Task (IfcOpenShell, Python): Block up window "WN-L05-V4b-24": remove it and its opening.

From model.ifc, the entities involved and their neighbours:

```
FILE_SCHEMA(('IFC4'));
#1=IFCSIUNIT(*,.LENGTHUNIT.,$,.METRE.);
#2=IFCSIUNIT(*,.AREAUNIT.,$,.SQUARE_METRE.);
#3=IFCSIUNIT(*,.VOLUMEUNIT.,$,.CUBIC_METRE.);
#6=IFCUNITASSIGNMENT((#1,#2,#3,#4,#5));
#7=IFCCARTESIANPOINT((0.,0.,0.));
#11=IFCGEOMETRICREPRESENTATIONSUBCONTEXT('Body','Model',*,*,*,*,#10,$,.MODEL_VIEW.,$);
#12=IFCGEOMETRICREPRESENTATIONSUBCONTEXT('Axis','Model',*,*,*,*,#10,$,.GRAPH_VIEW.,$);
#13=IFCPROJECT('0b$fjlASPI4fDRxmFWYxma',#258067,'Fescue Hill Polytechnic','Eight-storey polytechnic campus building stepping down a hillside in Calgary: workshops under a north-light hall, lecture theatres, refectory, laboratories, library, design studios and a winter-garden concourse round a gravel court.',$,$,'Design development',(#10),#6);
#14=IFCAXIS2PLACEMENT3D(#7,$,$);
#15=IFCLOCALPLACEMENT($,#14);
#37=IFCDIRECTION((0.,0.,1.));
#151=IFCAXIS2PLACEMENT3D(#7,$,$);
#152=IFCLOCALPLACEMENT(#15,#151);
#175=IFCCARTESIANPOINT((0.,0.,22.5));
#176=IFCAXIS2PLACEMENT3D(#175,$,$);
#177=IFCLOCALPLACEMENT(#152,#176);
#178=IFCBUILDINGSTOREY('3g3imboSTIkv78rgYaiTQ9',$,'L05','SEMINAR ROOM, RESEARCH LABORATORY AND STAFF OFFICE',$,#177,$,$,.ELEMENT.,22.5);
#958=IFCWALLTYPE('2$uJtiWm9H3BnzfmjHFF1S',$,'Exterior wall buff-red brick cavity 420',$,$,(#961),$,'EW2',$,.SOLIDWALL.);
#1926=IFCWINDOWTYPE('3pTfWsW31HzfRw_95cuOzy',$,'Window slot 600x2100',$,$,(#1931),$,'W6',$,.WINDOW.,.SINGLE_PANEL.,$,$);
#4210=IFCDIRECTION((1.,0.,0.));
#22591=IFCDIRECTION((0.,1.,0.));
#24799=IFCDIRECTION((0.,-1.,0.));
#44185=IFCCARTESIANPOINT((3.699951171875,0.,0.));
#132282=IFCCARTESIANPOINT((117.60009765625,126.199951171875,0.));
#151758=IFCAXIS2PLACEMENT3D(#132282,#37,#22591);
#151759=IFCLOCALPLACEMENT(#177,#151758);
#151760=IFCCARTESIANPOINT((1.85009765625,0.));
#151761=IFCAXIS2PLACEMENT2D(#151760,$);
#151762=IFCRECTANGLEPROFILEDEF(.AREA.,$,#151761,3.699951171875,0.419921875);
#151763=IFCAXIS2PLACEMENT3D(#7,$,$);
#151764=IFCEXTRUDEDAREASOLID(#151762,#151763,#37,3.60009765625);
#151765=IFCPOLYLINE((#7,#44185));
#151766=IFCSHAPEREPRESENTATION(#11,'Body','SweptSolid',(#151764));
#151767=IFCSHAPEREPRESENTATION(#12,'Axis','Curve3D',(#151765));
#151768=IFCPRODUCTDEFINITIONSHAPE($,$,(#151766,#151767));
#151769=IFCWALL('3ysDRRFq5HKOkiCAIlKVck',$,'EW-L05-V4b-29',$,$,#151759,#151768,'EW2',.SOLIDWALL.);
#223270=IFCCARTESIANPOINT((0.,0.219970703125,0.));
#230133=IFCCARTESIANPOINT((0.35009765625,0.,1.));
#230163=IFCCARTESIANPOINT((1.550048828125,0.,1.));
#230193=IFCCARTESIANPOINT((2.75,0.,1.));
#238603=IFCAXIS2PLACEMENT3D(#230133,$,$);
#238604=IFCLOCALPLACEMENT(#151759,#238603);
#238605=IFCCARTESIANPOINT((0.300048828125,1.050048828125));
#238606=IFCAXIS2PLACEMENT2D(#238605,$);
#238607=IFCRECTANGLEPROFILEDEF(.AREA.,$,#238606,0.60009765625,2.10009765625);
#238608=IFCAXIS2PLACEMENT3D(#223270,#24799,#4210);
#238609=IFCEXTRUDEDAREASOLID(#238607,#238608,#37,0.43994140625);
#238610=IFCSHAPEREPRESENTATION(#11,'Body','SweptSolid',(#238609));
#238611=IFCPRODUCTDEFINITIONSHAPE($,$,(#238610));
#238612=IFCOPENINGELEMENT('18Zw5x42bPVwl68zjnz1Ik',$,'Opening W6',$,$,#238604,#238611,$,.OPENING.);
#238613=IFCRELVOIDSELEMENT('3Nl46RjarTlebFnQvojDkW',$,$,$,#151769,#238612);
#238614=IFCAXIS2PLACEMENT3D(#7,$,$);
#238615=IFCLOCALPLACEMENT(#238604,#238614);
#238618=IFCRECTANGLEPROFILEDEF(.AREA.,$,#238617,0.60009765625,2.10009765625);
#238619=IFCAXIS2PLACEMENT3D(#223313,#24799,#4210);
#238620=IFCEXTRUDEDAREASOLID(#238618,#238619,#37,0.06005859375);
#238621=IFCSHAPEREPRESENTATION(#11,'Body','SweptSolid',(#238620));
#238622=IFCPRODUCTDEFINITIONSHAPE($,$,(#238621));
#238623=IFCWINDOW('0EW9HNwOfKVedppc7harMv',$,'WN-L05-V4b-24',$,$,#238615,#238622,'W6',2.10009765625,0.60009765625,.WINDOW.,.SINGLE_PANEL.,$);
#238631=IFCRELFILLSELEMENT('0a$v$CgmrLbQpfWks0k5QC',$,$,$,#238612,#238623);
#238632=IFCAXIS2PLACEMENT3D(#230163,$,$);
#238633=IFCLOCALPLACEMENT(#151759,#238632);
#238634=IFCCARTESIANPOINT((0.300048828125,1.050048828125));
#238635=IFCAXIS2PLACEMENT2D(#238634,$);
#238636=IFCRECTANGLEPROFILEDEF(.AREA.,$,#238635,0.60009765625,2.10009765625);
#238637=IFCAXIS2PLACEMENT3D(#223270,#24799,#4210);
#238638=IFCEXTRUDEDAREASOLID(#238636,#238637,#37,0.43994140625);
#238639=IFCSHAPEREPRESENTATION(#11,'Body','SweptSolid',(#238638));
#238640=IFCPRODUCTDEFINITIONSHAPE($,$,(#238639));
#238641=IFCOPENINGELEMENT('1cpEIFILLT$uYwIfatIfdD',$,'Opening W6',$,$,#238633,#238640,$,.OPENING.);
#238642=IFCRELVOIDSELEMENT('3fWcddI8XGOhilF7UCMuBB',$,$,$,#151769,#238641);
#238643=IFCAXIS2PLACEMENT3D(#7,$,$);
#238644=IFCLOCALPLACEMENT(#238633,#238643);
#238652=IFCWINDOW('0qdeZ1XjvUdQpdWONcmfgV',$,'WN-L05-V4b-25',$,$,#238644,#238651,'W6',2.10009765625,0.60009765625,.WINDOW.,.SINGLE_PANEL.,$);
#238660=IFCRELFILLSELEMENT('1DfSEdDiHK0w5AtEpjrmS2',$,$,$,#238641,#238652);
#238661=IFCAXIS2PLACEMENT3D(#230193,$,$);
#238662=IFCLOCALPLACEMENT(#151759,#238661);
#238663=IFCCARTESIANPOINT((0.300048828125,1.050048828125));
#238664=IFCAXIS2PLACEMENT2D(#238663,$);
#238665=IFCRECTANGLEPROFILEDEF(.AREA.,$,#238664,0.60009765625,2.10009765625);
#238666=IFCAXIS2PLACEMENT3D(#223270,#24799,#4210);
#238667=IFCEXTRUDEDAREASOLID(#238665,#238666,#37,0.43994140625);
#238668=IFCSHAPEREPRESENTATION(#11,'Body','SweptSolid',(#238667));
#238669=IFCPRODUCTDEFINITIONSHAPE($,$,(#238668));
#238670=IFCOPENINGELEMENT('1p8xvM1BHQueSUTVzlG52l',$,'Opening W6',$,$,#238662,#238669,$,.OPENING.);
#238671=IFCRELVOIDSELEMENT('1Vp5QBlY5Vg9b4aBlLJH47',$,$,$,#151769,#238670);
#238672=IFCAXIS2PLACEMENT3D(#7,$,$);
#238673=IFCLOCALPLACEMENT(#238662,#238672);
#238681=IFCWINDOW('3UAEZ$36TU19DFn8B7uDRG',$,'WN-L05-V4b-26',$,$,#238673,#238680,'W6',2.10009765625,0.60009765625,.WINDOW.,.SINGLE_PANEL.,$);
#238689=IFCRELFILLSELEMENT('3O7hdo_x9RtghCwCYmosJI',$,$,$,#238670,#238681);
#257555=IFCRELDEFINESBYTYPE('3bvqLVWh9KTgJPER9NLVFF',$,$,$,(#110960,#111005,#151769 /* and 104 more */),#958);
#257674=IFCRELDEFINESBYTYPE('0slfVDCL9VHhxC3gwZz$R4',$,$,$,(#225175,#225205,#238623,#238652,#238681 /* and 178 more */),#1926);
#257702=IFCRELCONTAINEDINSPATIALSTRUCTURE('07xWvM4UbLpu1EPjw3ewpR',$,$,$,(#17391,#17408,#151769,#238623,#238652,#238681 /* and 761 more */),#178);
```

```python
import ifcopenshell
import ifcopenshell.api.feature
import ifcopenshell.api.root
import ifcopenshell.geom
import ifcopenshell.util.shape

model = ifcopenshell.open("model.ifc")
settings = ifcopenshell.geom.settings()


def volume(element):
    """Net volume in cubic metres, openings subtracted."""
    shape = ifcopenshell.geom.create_shape(settings, element)
    return ifcopenshell.util.shape.get_volume(shape.geometry)


window = model.by_id(238623)
opening = window.FillsVoids[0].RelatingOpeningElement
wall = opening.VoidsElements[0].RelatingBuildingElement
before = volume(wall)

ifcopenshell.api.root.remove_product(model, product=window)
ifcopenshell.api.feature.remove_feature(model, feature=opening)

after = volume(wall)

print(f"wall volume {before:.3f} -> {after:.3f} m3")

model.write("model_edited.ifc")
```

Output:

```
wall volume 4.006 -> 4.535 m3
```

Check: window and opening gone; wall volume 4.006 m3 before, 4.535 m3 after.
